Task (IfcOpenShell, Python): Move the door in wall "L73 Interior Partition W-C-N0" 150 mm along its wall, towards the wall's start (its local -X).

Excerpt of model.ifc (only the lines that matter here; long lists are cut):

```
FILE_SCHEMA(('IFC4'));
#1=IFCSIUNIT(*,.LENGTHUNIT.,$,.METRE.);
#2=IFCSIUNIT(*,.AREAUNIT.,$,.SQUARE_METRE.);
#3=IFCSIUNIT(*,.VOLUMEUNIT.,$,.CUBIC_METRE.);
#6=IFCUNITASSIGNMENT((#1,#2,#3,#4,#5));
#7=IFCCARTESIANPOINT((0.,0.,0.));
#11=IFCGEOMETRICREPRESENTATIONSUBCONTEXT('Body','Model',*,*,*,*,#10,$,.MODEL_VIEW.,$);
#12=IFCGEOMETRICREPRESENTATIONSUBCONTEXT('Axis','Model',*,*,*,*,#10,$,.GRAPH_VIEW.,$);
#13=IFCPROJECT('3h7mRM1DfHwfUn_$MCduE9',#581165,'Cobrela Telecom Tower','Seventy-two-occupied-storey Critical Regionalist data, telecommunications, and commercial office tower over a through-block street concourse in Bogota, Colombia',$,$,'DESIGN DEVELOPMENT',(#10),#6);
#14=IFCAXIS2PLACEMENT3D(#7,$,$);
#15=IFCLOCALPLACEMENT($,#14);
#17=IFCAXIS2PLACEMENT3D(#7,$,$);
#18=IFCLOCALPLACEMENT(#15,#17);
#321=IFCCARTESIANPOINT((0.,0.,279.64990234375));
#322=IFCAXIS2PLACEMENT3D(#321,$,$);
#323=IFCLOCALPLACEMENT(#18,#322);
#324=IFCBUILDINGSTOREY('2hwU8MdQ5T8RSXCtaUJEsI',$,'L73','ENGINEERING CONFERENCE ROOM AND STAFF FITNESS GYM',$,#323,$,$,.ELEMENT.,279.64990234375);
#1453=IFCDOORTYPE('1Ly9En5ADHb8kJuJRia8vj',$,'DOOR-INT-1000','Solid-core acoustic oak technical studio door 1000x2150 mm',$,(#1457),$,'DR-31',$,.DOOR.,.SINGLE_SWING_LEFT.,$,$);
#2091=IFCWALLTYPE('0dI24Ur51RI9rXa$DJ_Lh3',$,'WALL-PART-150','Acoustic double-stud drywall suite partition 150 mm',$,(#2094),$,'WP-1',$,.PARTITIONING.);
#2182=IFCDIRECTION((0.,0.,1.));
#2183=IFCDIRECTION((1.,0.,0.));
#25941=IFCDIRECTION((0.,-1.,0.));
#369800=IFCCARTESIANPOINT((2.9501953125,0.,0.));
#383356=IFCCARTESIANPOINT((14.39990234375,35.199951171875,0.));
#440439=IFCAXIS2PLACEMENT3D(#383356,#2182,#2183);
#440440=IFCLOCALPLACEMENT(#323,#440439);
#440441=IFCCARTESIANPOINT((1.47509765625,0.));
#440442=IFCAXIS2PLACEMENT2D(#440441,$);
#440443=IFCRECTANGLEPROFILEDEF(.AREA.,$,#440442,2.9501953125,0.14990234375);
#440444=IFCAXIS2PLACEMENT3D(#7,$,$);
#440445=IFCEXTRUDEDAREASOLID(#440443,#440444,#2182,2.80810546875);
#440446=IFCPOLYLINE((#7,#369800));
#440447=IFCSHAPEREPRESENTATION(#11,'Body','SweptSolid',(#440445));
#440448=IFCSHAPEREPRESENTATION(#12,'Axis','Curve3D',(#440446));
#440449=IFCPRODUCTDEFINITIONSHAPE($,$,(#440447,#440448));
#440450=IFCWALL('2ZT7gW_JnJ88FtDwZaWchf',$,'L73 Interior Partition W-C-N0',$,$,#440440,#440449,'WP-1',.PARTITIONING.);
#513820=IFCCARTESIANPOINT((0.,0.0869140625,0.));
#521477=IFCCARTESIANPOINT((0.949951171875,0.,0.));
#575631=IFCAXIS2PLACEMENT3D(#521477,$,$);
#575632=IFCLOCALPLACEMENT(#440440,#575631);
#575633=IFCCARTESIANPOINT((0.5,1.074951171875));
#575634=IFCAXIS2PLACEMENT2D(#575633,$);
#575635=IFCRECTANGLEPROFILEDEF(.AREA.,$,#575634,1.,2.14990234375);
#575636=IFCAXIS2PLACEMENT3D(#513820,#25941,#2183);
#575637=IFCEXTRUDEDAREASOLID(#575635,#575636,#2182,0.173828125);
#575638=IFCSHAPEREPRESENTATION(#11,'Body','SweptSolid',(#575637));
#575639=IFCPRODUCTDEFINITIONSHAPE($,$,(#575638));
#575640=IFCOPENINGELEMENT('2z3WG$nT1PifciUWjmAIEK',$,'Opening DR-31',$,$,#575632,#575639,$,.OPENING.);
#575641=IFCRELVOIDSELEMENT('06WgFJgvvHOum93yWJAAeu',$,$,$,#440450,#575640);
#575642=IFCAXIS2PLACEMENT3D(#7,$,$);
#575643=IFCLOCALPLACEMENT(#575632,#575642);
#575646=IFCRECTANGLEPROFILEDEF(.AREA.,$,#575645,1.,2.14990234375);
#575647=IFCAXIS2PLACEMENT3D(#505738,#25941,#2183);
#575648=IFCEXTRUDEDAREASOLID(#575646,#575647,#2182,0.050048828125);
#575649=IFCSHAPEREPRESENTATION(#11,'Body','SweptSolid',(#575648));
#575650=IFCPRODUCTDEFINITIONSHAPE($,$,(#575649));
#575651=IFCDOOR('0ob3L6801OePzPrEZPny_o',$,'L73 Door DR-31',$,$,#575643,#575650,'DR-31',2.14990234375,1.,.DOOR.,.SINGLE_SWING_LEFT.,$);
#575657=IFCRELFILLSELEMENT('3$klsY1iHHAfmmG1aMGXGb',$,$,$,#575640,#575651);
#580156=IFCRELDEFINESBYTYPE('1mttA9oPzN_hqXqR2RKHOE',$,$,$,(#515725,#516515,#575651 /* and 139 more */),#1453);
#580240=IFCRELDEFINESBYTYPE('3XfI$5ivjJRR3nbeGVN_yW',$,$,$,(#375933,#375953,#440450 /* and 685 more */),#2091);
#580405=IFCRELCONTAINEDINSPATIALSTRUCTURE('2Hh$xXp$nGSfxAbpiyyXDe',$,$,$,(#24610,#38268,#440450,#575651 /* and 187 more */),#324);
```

```python
import ifcopenshell
import ifcopenshell.api.geometry
import ifcopenshell.util.placement

model = ifcopenshell.open("model.ifc")

door = model.by_id(575651)
opening = door.FillsVoids[0].RelatingOpeningElement
wall = opening.VoidsElements[0].RelatingBuildingElement

wall_matrix = ifcopenshell.util.placement.get_local_placement(wall.ObjectPlacement)
shift = wall_matrix[:3, 0] * -0.15
before = ifcopenshell.util.placement.get_local_placement(door.ObjectPlacement)[:3, 3].copy()

# The door is placed relative to its opening, so it follows when the opening moves.
matrix = ifcopenshell.util.placement.get_local_placement(opening.ObjectPlacement)
matrix[:3, 3] += shift
ifcopenshell.api.geometry.edit_object_placement(
    model, product=opening, matrix=matrix, is_si=False, should_transform_children=True
)

after = ifcopenshell.util.placement.get_local_placement(door.ObjectPlacement)[:3, 3]
print("door moved by", (after - before).round(3) + 0.0)

model.write("model_updated.ifc")
```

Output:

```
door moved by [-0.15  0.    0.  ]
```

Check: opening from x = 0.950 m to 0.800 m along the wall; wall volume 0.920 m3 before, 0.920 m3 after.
